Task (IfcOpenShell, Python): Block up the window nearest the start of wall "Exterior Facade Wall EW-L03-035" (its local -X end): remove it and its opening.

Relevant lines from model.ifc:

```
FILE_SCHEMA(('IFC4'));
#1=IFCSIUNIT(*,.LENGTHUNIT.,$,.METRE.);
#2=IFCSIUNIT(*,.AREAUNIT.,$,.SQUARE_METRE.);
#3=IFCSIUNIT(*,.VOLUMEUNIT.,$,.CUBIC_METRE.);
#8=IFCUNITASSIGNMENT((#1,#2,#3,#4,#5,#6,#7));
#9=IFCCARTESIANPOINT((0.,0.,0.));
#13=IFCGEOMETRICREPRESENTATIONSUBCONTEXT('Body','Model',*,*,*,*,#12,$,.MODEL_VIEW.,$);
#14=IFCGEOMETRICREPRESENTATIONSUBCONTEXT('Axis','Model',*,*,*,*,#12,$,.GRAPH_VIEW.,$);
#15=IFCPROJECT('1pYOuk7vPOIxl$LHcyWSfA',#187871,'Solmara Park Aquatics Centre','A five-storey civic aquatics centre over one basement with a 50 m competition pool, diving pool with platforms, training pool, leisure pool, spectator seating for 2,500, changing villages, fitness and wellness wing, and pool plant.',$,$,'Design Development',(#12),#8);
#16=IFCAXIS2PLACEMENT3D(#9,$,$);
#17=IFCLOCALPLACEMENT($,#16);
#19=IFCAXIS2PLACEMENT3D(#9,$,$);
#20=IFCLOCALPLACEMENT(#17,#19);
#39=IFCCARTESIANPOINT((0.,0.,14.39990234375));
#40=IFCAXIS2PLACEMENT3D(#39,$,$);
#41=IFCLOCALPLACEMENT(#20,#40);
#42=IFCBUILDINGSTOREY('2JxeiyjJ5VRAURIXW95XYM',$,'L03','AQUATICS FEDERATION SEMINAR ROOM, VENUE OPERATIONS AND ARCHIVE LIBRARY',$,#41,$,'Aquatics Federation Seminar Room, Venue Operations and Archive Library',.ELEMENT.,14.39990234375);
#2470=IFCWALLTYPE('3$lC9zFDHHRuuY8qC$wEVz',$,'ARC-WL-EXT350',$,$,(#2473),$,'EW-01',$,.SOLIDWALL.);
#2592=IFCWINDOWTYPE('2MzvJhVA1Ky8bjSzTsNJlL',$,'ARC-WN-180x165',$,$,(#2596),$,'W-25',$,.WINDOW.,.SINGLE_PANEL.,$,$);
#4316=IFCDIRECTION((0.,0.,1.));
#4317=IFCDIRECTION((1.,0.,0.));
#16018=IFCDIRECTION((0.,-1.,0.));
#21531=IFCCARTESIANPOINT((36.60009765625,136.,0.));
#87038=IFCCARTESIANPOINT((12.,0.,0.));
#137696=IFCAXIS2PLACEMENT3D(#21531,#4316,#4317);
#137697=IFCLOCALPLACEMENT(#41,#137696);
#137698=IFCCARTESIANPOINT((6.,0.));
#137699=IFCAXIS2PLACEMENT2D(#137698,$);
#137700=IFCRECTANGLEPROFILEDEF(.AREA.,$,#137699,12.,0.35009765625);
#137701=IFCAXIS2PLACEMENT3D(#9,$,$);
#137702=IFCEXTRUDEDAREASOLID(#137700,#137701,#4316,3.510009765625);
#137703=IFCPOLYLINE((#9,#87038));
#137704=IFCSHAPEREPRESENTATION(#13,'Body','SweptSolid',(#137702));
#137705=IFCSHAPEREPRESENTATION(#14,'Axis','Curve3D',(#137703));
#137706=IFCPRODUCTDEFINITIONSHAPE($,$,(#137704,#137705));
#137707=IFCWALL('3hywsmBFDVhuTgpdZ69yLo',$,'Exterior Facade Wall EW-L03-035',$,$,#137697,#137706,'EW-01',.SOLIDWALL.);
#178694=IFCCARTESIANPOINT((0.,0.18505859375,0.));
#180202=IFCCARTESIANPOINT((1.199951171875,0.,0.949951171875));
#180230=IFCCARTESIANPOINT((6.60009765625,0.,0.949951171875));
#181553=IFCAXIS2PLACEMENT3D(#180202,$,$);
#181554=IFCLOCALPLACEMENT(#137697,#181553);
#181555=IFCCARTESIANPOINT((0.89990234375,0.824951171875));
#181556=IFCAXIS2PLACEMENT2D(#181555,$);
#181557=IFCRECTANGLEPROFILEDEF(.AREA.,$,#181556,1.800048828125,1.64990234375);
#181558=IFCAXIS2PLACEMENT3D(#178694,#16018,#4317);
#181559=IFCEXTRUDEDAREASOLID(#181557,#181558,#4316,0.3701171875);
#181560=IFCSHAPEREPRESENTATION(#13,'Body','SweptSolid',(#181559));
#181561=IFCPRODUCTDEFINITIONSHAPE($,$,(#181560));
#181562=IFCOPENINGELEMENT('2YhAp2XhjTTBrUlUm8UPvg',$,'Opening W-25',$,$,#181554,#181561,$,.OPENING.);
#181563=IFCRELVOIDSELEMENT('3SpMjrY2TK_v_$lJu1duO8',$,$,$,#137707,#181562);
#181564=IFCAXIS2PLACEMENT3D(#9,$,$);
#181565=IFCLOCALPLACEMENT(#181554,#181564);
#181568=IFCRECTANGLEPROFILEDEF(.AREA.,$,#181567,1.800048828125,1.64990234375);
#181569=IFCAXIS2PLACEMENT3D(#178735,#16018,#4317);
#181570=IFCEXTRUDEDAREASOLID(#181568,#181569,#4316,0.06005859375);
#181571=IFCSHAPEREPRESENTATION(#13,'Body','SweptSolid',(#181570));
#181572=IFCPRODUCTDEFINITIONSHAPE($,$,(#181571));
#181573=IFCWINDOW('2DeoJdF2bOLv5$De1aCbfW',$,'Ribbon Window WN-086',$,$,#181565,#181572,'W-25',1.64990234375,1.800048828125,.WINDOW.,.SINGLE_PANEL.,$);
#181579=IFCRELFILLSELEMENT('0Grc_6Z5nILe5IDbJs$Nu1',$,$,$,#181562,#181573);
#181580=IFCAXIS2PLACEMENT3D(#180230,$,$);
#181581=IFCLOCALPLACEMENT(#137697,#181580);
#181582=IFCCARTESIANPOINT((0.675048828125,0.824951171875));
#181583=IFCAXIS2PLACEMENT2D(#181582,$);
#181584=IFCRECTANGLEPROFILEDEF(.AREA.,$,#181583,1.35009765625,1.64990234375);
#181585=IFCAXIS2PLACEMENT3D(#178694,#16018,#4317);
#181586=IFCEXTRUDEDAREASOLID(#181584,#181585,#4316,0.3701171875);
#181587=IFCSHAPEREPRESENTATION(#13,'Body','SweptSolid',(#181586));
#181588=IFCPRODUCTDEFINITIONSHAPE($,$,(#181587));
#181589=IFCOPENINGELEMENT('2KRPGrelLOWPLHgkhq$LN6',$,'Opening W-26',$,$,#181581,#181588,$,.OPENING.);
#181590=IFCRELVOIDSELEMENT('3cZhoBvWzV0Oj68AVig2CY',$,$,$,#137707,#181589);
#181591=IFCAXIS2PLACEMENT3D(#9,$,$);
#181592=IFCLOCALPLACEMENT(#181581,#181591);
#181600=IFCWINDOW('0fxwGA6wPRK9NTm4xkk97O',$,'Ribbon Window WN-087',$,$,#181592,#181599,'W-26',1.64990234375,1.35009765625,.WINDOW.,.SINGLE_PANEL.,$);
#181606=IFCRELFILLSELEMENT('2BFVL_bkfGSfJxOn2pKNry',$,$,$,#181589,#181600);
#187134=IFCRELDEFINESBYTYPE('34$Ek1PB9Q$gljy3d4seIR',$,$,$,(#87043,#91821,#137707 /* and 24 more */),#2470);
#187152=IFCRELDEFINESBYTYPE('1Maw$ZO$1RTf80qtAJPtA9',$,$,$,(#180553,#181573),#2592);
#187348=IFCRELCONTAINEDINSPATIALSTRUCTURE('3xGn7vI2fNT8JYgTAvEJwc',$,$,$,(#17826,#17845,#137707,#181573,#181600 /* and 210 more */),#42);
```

```python
import ifcopenshell
import ifcopenshell.api.feature
import ifcopenshell.api.root
import ifcopenshell.geom
import ifcopenshell.util.shape

model = ifcopenshell.open("model.ifc")
settings = ifcopenshell.geom.settings()


def volume(element):
    """Net volume in cubic metres, openings subtracted."""
    shape = ifcopenshell.geom.create_shape(settings, element)
    return ifcopenshell.util.shape.get_volume(shape.geometry)


window = model.by_id(181573)
opening = window.FillsVoids[0].RelatingOpeningElement
wall = opening.VoidsElements[0].RelatingBuildingElement
before = volume(wall)

ifcopenshell.api.root.remove_product(model, product=window)
ifcopenshell.api.feature.remove_feature(model, feature=opening)

after = volume(wall)

print(f"wall volume {before:.3f} -> {after:.3f} m3")

model.write("model-out.ifc")
```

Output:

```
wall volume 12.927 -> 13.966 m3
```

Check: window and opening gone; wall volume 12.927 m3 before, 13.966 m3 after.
